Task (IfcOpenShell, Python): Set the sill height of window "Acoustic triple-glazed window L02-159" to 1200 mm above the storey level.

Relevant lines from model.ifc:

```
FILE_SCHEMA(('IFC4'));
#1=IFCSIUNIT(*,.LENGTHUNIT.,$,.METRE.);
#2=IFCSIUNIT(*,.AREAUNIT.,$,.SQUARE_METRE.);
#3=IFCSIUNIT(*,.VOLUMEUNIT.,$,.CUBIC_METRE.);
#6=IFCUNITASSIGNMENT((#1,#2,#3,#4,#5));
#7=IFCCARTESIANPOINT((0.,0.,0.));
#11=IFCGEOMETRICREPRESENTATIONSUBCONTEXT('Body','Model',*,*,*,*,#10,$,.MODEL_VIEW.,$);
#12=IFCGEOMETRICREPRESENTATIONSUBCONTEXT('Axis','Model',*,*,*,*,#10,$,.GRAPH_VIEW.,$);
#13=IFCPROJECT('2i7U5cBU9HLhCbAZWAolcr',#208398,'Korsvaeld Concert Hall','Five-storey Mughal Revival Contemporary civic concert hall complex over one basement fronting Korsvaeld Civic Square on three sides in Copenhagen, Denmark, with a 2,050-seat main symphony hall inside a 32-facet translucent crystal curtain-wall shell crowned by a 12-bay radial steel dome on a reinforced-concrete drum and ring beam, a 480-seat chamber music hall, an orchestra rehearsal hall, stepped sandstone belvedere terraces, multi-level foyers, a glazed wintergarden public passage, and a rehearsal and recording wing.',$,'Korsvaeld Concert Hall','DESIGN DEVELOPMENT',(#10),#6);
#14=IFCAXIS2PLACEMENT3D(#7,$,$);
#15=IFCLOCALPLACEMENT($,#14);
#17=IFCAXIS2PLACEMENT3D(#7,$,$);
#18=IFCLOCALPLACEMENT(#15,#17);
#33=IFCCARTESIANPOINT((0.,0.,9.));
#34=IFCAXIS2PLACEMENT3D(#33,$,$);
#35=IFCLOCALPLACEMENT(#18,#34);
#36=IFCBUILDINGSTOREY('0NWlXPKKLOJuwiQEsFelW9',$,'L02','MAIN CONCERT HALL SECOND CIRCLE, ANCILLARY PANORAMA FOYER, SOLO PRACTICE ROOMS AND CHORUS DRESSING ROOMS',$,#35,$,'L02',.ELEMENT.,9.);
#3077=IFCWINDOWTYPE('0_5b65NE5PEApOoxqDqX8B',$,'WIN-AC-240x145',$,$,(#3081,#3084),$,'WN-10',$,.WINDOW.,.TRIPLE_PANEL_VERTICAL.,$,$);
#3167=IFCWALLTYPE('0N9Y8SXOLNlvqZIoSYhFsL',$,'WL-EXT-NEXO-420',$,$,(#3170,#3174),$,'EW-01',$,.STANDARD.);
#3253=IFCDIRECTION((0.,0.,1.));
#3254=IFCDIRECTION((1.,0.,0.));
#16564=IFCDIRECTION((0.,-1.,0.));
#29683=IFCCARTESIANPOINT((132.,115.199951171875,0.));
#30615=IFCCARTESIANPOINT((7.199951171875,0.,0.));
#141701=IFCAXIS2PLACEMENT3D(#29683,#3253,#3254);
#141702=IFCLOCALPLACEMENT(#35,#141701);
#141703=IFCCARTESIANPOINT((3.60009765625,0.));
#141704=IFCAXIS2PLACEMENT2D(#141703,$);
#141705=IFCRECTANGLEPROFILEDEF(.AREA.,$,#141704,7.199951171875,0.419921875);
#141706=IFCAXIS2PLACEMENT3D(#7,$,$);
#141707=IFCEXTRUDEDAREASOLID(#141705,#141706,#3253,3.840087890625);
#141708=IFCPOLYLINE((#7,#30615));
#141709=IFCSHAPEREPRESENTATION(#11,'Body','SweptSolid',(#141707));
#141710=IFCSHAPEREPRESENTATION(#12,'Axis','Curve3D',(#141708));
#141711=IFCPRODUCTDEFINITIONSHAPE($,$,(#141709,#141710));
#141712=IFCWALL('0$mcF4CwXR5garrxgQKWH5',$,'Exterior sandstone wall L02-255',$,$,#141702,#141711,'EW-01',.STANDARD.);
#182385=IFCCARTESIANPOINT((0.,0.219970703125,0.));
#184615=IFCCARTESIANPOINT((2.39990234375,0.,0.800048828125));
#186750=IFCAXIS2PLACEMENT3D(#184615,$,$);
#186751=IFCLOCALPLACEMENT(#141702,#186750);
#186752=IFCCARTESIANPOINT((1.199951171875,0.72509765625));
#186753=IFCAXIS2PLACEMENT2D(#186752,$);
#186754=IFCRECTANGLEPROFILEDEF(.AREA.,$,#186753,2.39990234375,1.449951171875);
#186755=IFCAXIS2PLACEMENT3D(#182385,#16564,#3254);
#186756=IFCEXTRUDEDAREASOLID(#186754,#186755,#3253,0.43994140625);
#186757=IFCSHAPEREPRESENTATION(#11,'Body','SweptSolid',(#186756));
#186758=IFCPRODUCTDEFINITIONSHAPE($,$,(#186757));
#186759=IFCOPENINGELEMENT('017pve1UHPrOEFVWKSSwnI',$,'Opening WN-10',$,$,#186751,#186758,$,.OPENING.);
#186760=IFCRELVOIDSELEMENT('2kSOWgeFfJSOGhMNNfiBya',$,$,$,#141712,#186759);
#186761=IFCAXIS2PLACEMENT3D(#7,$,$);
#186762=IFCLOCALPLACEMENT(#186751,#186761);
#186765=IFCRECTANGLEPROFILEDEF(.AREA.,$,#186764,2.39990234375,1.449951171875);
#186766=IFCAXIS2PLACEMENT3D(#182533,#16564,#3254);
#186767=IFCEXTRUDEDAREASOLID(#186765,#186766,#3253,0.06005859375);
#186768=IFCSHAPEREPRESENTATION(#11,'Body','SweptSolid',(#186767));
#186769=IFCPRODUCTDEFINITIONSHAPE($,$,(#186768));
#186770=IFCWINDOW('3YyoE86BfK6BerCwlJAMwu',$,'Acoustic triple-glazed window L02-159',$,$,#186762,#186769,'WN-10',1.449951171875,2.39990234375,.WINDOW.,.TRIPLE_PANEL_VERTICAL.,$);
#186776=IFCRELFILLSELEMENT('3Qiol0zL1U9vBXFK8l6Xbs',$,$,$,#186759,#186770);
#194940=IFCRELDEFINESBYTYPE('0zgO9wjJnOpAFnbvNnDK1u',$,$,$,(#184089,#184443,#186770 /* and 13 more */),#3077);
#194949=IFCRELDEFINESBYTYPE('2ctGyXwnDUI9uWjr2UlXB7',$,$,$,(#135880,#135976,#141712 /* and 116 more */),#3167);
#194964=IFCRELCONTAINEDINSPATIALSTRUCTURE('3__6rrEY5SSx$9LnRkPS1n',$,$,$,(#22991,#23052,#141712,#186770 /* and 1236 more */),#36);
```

```python
import numpy as np
import ifcopenshell
import ifcopenshell.api.geometry
import ifcopenshell.geom
import ifcopenshell.util.element
import ifcopenshell.util.placement
import ifcopenshell.util.shape
import ifcopenshell.util.unit

model = ifcopenshell.open("model.ifc")
unit_scale = ifcopenshell.util.unit.calculate_unit_scale(model)

window = model.by_guid("3YyoE86BfK6BerCwlJAMwu")
opening = window.FillsVoids[0].RelatingOpeningElement
storey = ifcopenshell.util.element.get_container(window, ifc_class="IfcBuildingStorey")
level = ifcopenshell.util.placement.get_local_placement(storey.ObjectPlacement)[2, 3]

# The opening's origin need not be at the sill, so measure its lowest point.
shape = ifcopenshell.geom.create_shape(ifcopenshell.geom.settings(), opening)
bottom = ifcopenshell.util.shape.get_shape_bottom_elevation(shape, shape.geometry) / unit_scale
dz = level + 1.2 / unit_scale - bottom

shift = np.array([0.0, 0.0, dz])
# The window is placed relative to its opening, so it follows when the opening moves.
matrix = ifcopenshell.util.placement.get_local_placement(opening.ObjectPlacement)
matrix[:3, 3] += shift
ifcopenshell.api.geometry.edit_object_placement(
    model, product=opening, matrix=matrix, is_si=False, should_transform_children=True
)

print(f"moved by {dz * unit_scale:+.3f} m")

model.write("model-out.ifc")
```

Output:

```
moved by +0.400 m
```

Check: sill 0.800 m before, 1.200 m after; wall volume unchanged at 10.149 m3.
